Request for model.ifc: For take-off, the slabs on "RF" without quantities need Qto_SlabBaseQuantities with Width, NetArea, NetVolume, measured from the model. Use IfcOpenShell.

First a look at what the model holds.

```python
import ifcopenshell
import ifcopenshell.util.element
import ifcopenshell.util.unit

model = ifcopenshell.open("model.ifc")
print(model.schema)
for unit_type in ("LENGTHUNIT", "AREAUNIT", "VOLUMEUNIT"):
    print(unit_type, ifcopenshell.util.unit.calculate_unit_scale(model, unit_type))
storey = next(s for s in model.by_type("IfcBuildingStorey") if s.Name == "RF")
slabs = [e for e in ifcopenshell.util.element.get_decomposition(storey) if e.is_a("IfcSlab")]
for e in sorted(slabs, key=lambda e: e.id()):
    print(e.id(), e.is_a(), e.Name, list(ifcopenshell.util.element.get_psets(e, qtos_only=True)), sep=" | ")
```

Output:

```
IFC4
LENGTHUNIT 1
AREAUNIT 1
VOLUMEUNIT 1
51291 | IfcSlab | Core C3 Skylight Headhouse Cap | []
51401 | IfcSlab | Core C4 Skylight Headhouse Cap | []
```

```python
import ifcopenshell
import ifcopenshell.api.pset
import ifcopenshell.geom
import ifcopenshell.util.element
import ifcopenshell.util.shape
import ifcopenshell.util.unit

model = ifcopenshell.open("model.ifc")
unit_scale = ifcopenshell.util.unit.calculate_unit_scale(model)
area_scale = ifcopenshell.util.unit.calculate_unit_scale(model, "AREAUNIT")
volume_scale = ifcopenshell.util.unit.calculate_unit_scale(model, "VOLUMEUNIT")
settings = ifcopenshell.geom.settings()

storey = next(s for s in model.by_type("IfcBuildingStorey") if s.Name == "RF")
slabs = [e for e in ifcopenshell.util.element.get_decomposition(storey) if e.is_a("IfcSlab")]

for e in sorted(slabs, key=lambda e: e.id()):
    if ifcopenshell.util.element.get_psets(e, qtos_only=True, should_inherit=False):
        continue
    # Geometry comes back in metres, in the element's own axes.
    shape = ifcopenshell.geom.create_shape(settings, e)
    values = {
        "Width": ifcopenshell.util.shape.get_z(shape.geometry) / unit_scale,
        "NetArea": ifcopenshell.util.shape.get_footprint_area(shape.geometry) / area_scale,
        "NetVolume": ifcopenshell.util.shape.get_volume(shape.geometry) / volume_scale,
    }
    qto = ifcopenshell.api.pset.add_qto(model, product=e, name="Qto_SlabBaseQuantities")
    ifcopenshell.api.pset.edit_qto(model, qto=qto, properties=values)
    print(e.id(), {k: round(v, 3) for k, v in values.items()})

model.write("model_updated.ifc")
```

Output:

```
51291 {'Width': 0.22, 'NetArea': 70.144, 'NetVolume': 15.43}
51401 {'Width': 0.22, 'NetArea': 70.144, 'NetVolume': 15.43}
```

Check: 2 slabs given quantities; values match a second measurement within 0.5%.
